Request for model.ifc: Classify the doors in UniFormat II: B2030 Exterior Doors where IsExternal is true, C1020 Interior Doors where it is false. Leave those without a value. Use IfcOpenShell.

First a look at what the model holds.

```python
import ifcopenshell
import ifcopenshell.util.element

model = ifcopenshell.open("model.ifc")
print(model.schema)
print("classifications:", [c.Name for c in model.by_type("IfcClassification")])
values = [ifcopenshell.util.element.get_pset(e, "Pset_DoorCommon", "IsExternal") for e in model.by_type("IfcDoor")]
for value in (True, False, None):
    print("IsExternal", value, values.count(value))
```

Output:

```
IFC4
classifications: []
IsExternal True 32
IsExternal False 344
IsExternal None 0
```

```python
import ifcopenshell
import ifcopenshell.api.classification
import ifcopenshell.util.element

model = ifcopenshell.open("model.ifc")

system = ifcopenshell.api.classification.add_classification(model, classification="UniFormat II")

doors = model.by_type("IfcDoor")
external = {e: ifcopenshell.util.element.get_pset(e, "Pset_DoorCommon", "IsExternal") for e in doors}
for flag, code, name in ((True, "B2030", "Exterior Doors"), (False, "C1020", "Interior Doors")):
    products = [e for e in doors if external[e] is flag]
    ifcopenshell.api.classification.add_reference(
        model, products=products, classification=system, identification=code, name=name
    )
    print(code, len(products))

model.write("model_updated.ifc")
```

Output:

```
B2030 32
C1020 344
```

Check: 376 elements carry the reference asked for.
